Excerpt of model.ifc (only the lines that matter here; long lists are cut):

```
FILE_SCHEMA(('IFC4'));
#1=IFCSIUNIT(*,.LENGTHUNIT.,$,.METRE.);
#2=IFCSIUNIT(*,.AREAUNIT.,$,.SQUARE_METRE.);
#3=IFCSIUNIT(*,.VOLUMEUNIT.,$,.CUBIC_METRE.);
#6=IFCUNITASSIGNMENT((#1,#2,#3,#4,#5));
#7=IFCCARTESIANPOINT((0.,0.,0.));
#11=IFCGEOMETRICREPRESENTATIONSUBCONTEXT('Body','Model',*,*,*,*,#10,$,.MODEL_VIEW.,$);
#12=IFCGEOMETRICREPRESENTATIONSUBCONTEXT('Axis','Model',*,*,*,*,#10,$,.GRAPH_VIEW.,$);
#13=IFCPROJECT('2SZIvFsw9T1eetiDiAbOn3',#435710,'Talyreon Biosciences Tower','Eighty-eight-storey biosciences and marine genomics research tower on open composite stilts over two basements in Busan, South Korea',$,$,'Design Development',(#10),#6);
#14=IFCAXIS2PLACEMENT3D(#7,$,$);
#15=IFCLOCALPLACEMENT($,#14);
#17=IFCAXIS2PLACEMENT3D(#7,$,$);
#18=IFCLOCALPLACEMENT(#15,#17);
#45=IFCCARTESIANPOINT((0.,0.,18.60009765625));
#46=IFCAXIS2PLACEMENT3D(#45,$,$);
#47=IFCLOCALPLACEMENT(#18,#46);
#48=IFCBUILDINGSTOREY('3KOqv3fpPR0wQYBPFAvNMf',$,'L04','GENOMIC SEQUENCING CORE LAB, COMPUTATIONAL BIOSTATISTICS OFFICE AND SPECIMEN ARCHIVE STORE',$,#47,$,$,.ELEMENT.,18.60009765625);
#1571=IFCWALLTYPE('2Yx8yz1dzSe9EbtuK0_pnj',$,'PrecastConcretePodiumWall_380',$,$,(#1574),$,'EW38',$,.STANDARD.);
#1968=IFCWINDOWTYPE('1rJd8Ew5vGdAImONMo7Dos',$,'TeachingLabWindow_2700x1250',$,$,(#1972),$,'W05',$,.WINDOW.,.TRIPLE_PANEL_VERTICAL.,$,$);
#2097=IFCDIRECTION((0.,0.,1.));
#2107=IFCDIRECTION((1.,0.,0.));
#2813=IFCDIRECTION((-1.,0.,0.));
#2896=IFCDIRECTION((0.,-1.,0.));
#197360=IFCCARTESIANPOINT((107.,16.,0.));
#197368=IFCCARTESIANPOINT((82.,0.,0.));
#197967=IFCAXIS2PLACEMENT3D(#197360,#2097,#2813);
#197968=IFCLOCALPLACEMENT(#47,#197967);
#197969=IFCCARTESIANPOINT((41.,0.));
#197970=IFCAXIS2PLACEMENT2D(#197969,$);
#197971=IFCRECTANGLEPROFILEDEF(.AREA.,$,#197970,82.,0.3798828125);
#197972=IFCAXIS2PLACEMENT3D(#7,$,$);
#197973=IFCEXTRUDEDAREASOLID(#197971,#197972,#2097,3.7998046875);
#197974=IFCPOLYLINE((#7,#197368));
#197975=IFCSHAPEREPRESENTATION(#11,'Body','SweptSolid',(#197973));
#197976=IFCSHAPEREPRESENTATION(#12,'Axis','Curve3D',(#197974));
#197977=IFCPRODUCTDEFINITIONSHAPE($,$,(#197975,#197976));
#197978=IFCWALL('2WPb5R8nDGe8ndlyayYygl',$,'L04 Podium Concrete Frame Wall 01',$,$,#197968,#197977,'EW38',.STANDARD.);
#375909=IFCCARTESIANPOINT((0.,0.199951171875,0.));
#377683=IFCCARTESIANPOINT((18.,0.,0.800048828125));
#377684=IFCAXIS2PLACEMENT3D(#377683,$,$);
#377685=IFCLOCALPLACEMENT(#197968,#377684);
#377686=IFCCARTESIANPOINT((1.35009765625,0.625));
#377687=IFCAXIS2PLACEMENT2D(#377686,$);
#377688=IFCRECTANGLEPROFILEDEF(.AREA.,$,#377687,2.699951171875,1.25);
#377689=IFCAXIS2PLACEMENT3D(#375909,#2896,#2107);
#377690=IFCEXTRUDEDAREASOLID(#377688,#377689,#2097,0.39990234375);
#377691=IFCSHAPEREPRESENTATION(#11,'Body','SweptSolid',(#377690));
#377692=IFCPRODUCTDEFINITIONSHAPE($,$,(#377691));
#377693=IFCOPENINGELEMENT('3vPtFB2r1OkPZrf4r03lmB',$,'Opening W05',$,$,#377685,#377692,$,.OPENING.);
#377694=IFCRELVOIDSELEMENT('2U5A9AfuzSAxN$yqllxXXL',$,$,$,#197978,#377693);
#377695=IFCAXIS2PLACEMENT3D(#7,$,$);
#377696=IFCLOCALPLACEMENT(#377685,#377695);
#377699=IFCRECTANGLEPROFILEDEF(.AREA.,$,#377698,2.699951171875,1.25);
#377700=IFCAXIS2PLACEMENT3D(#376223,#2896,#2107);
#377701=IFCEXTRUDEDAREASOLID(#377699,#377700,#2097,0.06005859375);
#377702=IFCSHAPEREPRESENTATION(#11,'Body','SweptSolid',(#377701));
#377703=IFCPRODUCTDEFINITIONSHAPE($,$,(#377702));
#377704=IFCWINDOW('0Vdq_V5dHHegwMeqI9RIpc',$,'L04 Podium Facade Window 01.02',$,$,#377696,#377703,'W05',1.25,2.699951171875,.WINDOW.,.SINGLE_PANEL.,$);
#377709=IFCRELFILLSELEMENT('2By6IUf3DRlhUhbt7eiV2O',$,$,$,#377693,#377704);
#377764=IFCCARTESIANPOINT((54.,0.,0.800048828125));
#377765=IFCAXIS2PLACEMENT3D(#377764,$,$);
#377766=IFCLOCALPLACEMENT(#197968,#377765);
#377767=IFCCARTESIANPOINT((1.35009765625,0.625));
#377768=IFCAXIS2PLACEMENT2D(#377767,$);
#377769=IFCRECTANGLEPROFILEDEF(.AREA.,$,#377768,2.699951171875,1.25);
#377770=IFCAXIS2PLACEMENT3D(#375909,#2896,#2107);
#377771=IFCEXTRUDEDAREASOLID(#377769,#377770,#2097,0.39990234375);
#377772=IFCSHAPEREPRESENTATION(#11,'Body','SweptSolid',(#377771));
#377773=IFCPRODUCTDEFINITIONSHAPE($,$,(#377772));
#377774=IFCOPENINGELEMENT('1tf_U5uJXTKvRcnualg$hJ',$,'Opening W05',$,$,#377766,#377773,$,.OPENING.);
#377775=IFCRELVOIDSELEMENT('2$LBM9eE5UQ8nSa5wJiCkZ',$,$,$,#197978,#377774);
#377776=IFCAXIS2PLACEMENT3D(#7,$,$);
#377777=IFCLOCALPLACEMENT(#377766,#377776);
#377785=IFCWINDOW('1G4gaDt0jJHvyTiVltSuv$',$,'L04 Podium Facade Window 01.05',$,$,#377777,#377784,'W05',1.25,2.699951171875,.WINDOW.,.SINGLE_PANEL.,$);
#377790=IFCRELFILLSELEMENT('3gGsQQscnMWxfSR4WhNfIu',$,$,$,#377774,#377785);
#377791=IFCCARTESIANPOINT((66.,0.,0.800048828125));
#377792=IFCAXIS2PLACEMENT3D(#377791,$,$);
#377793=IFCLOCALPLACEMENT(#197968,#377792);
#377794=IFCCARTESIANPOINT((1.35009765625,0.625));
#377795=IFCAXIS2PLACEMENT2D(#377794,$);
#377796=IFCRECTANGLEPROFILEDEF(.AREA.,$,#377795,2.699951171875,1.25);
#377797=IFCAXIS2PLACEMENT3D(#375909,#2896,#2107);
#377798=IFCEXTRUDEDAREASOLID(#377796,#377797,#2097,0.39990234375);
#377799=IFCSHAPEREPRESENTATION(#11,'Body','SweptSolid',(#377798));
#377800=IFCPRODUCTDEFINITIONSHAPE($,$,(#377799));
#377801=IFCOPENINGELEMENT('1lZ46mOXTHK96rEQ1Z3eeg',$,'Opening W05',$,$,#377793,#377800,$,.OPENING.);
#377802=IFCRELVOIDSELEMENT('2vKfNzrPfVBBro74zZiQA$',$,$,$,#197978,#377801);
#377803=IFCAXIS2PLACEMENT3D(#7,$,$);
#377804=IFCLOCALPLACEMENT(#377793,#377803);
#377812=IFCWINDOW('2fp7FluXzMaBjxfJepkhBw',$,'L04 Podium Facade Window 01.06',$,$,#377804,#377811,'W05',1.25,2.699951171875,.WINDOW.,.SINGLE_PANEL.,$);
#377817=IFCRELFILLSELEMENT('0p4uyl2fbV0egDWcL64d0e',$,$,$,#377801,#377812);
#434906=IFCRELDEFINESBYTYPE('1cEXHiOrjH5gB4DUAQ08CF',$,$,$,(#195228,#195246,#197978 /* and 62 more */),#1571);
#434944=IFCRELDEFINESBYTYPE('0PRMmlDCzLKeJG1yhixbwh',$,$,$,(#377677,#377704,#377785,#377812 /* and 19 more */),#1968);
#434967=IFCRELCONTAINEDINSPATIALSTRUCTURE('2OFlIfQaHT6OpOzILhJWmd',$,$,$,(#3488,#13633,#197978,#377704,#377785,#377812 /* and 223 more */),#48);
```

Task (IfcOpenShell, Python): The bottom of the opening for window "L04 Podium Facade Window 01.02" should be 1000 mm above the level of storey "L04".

```python
import numpy as np
import ifcopenshell
import ifcopenshell.api.geometry
import ifcopenshell.geom
import ifcopenshell.util.element
import ifcopenshell.util.placement
import ifcopenshell.util.shape
import ifcopenshell.util.unit

model = ifcopenshell.open("model.ifc")
unit_scale = ifcopenshell.util.unit.calculate_unit_scale(model)

window = model.by_guid("0Vdq_V5dHHegwMeqI9RIpc")
opening = window.FillsVoids[0].RelatingOpeningElement
storey = ifcopenshell.util.element.get_container(window, ifc_class="IfcBuildingStorey")
level = ifcopenshell.util.placement.get_local_placement(storey.ObjectPlacement)[2, 3]

# The opening's origin need not be at the sill, so measure its lowest point.
shape = ifcopenshell.geom.create_shape(ifcopenshell.geom.settings(), opening)
bottom = ifcopenshell.util.shape.get_shape_bottom_elevation(shape, shape.geometry) / unit_scale
dz = level + 1 / unit_scale - bottom

shift = np.array([0.0, 0.0, dz])
# The window is placed relative to its opening, so it follows when the opening moves.
matrix = ifcopenshell.util.placement.get_local_placement(opening.ObjectPlacement)
matrix[:3, 3] += shift
ifcopenshell.api.geometry.edit_object_placement(
    model, product=opening, matrix=matrix, is_si=False, should_transform_children=True
)

print(f"moved by {dz * unit_scale:+.3f} m")

model.write("model_v2.ifc")
```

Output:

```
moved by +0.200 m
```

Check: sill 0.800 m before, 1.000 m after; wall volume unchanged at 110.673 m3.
